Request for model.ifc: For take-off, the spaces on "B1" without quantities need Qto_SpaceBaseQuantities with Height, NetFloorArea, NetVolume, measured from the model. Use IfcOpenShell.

First a look at what the model holds.

```python
import ifcopenshell
import ifcopenshell.util.element
import ifcopenshell.util.unit

model = ifcopenshell.open("model.ifc")
print(model.schema)
for unit_type in ("LENGTHUNIT", "AREAUNIT", "VOLUMEUNIT"):
    print(unit_type, ifcopenshell.util.unit.calculate_unit_scale(model, unit_type))
storey = next(s for s in model.by_type("IfcBuildingStorey") if s.Name == "B1")
spaces = [e for e in ifcopenshell.util.element.get_decomposition(storey) if e.is_a("IfcSpace")]
for e in sorted(spaces, key=lambda e: e.id()):
    print(e.id(), e.is_a(), e.Name, list(ifcopenshell.util.element.get_psets(e, qtos_only=True)), sep=" | ")
```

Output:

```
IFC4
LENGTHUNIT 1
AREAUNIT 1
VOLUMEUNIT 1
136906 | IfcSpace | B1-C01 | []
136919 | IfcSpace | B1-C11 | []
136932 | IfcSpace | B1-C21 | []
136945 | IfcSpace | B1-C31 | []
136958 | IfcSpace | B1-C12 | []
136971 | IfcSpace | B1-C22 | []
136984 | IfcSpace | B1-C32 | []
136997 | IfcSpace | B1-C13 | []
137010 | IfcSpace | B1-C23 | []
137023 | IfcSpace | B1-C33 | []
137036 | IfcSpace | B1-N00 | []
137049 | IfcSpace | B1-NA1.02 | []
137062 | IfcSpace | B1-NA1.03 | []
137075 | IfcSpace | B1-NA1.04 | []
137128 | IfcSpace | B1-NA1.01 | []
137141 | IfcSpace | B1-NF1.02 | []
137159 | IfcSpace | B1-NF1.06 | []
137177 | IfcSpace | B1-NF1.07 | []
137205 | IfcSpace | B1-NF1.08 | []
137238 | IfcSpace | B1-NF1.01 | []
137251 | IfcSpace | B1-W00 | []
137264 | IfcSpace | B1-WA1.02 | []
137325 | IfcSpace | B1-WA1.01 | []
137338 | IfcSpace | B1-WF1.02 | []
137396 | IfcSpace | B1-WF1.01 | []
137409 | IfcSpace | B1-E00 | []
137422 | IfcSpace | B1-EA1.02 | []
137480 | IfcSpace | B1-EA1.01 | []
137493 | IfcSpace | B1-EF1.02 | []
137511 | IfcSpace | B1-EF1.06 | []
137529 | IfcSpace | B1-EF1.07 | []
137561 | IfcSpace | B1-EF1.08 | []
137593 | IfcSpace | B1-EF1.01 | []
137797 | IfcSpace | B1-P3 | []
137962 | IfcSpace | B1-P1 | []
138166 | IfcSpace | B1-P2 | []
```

```python
import ifcopenshell
import ifcopenshell.api.pset
import ifcopenshell.geom
import ifcopenshell.util.element
import ifcopenshell.util.shape
import ifcopenshell.util.unit

model = ifcopenshell.open("model.ifc")
unit_scale = ifcopenshell.util.unit.calculate_unit_scale(model)
area_scale = ifcopenshell.util.unit.calculate_unit_scale(model, "AREAUNIT")
volume_scale = ifcopenshell.util.unit.calculate_unit_scale(model, "VOLUMEUNIT")
settings = ifcopenshell.geom.settings()

storey = next(s for s in model.by_type("IfcBuildingStorey") if s.Name == "B1")
spaces = [e for e in ifcopenshell.util.element.get_decomposition(storey) if e.is_a("IfcSpace")]

for e in sorted(spaces, key=lambda e: e.id()):
    if ifcopenshell.util.element.get_psets(e, qtos_only=True, should_inherit=False):
        continue
    # Geometry comes back in metres, in the element's own axes.
    shape = ifcopenshell.geom.create_shape(settings, e)
    values = {
        "Height": ifcopenshell.util.shape.get_z(shape.geometry) / unit_scale,
        "NetFloorArea": ifcopenshell.util.shape.get_footprint_area(shape.geometry) / area_scale,
        "NetVolume": ifcopenshell.util.shape.get_volume(shape.geometry) / volume_scale,
    }
    qto = ifcopenshell.api.pset.add_qto(model, product=e, name="Qto_SpaceBaseQuantities")
    ifcopenshell.api.pset.edit_qto(model, qto=qto, properties=values)
    print(e.id(), {k: round(v, 3) for k, v in values.items()})

model.write("model_rev.ifc")
```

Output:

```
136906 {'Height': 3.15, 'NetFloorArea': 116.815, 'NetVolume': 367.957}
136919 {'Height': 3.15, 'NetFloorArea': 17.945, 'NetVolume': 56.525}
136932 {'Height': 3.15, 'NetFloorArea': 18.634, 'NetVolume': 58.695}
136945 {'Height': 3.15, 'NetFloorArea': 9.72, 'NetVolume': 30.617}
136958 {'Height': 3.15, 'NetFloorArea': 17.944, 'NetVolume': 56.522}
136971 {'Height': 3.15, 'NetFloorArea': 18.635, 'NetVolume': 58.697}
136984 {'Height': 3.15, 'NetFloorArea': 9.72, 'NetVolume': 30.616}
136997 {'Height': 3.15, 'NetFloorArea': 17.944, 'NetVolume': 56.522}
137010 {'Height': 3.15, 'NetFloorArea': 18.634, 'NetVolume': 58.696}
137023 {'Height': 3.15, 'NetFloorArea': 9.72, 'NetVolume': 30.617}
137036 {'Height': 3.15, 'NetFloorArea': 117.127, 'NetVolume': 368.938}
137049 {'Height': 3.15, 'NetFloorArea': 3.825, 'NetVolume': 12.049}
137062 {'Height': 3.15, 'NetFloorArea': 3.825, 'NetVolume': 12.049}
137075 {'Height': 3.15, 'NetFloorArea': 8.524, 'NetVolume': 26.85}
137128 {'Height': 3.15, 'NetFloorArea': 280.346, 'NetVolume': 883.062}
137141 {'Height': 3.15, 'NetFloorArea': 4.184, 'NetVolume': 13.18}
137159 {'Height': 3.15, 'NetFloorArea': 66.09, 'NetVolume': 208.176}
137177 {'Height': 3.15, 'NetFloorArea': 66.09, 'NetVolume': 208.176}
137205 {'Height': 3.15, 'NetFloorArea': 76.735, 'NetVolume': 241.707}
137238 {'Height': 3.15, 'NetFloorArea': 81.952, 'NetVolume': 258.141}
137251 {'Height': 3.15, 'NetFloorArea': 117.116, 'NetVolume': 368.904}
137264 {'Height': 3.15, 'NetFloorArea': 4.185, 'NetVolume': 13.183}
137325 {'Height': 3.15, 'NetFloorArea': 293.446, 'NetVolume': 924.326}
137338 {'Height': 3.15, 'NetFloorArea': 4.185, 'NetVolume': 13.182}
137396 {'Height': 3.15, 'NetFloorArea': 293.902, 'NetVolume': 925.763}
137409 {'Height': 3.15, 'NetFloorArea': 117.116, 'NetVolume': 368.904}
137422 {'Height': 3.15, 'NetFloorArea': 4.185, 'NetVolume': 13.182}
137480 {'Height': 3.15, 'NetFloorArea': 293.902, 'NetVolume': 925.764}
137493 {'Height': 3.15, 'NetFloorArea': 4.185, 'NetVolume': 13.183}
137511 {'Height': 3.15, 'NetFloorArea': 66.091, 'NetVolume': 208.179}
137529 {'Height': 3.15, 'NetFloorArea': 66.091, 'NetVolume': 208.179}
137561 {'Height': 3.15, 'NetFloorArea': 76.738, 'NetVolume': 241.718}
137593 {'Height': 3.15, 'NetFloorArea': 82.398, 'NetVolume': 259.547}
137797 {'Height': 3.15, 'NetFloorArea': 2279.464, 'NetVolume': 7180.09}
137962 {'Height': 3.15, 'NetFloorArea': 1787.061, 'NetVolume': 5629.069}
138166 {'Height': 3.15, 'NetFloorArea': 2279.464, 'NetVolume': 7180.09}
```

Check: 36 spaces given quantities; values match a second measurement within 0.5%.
